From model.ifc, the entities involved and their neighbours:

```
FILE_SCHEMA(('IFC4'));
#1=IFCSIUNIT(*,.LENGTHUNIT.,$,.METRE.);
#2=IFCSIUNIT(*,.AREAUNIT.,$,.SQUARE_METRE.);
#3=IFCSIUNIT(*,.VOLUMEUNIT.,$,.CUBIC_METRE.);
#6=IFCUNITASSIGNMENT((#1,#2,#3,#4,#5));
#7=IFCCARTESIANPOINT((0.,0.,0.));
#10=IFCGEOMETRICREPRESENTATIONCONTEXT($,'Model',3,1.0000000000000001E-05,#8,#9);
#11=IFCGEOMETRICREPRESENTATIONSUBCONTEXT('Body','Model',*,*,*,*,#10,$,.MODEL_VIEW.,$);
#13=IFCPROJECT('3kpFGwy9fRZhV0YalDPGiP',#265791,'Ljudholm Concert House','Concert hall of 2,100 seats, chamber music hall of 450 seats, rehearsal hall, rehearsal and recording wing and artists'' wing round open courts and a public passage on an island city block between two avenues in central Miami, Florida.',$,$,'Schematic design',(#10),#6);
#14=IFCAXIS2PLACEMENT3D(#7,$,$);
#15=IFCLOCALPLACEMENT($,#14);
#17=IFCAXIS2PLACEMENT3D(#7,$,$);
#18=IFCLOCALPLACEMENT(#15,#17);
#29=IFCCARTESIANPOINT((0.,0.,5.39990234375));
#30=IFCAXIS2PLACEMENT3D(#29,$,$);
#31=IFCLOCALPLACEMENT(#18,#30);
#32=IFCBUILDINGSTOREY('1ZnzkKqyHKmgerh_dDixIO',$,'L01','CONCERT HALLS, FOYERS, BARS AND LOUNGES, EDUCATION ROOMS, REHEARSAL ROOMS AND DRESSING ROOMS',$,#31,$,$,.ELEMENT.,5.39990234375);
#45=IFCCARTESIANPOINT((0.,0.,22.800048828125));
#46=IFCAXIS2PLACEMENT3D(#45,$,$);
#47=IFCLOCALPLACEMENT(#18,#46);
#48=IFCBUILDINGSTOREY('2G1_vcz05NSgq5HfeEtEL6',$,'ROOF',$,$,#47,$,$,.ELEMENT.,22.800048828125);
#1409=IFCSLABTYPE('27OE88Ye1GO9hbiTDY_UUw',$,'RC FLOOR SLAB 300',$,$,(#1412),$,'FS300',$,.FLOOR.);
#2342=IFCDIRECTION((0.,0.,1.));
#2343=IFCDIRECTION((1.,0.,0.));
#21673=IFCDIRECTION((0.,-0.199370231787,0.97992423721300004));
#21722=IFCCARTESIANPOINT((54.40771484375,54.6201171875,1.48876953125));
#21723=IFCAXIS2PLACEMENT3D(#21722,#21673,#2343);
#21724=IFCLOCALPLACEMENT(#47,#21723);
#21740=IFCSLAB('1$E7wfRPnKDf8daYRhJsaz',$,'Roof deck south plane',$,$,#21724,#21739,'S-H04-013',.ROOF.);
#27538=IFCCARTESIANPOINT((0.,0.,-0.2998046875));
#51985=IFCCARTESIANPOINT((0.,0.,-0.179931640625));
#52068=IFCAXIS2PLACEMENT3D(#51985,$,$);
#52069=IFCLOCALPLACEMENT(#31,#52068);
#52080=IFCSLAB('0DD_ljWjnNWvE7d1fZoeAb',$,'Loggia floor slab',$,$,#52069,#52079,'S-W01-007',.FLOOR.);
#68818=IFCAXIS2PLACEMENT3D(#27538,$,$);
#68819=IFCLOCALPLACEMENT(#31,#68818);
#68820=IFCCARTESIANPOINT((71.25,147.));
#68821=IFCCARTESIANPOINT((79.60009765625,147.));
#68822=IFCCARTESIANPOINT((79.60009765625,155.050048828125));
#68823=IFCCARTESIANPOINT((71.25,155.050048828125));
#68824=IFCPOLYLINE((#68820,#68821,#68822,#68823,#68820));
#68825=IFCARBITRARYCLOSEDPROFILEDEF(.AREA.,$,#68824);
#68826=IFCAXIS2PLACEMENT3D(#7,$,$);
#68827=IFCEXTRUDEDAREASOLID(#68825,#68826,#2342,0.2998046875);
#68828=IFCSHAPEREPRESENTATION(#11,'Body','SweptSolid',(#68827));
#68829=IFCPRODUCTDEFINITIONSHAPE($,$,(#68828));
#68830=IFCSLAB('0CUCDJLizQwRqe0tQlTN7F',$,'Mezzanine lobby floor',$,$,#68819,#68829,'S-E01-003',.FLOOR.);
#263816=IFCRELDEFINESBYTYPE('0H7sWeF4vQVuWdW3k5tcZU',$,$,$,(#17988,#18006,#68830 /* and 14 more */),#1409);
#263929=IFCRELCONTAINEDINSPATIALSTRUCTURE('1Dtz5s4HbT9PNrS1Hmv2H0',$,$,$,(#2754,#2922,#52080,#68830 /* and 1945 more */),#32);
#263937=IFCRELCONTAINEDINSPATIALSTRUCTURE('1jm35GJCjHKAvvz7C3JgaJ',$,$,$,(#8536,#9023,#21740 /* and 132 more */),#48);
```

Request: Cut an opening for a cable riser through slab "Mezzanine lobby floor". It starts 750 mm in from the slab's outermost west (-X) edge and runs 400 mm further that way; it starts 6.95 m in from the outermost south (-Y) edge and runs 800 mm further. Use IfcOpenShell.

```python
import numpy as np
import ifcopenshell
import ifcopenshell.api.feature
import ifcopenshell.api.geometry
import ifcopenshell.api.root
import ifcopenshell.geom
import ifcopenshell.util.placement
import ifcopenshell.util.representation
import ifcopenshell.util.shape
import ifcopenshell.util.unit

model = ifcopenshell.open("model.ifc")
unit_scale = ifcopenshell.util.unit.calculate_unit_scale(model)
settings = ifcopenshell.geom.settings()


def volume(element):
    """Net volume in cubic metres, openings subtracted."""
    shape = ifcopenshell.geom.create_shape(settings, element)
    return ifcopenshell.util.shape.get_volume(shape.geometry)


slab = model.by_guid("0CUCDJLizQwRqe0tQlTN7F")
before = volume(slab)

# Extent in the slab's own axes, in metres. The edges named are its -X and -Y sides.
slab_shape = ifcopenshell.geom.create_shape(settings, slab)
vertices = ifcopenshell.util.shape.get_vertices(slab_shape.geometry)
x_min, y_min, bottom = vertices.min(axis=0)
top = vertices[:, 2].max()

opening = ifcopenshell.api.root.create_entity(model, ifc_class="IfcOpeningElement", name="Cable riser opening", predefined_type="OPENING")
context = ifcopenshell.util.representation.get_context(model, "Model", "Body", "MODEL_VIEW")
width, depth = 0.4, 0.8
outline = [(0.0, 0.0), (width, 0.0), (width, depth), (0.0, depth), (0.0, 0.0)]
# Overshoot both faces by 50 mm so the cut is clean.
shape = ifcopenshell.api.geometry.add_slab_representation(
    model, context=context, depth=top - bottom + 0.1, polyline=outline
)
ifcopenshell.api.geometry.assign_representation(model, product=opening, representation=shape)

matrix = ifcopenshell.util.placement.get_local_placement(slab.ObjectPlacement)
matrix[:, 3] = matrix @ np.append(np.array([x_min + 0.75, y_min + 6.95, bottom - 0.05]) / unit_scale, 1.0)
ifcopenshell.api.geometry.edit_object_placement(model, product=opening, matrix=matrix, is_si=False)
ifcopenshell.api.feature.add_feature(model, feature=opening, element=slab)

after = volume(slab)

print(f"slab volume {before:.3f} -> {after:.3f} m3")

model.write("model_updated.ifc")
```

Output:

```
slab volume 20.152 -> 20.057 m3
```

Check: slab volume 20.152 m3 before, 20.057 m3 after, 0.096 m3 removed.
